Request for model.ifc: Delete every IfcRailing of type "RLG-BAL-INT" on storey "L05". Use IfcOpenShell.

First a look at what the model holds.

```python
import ifcopenshell
import ifcopenshell.util.element

model = ifcopenshell.open("model.ifc")
print(model.schema)
storey = next(s for s in model.by_type("IfcBuildingStorey") if s.Name == "L05")
railings = [e for e in ifcopenshell.util.element.get_decomposition(storey) if e.is_a("IfcRailing")]
seen = {}
for e in railings:
    element_type = ifcopenshell.util.element.get_type(e)
    name = element_type.Name if element_type not in (None, e) else None
    seen[name] = seen.get(name, 0) + 1
for name, count in sorted(seen.items(), key=str):
    print(count, "x", name)
```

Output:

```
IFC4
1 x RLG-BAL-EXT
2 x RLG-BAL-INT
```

```python
import ifcopenshell
import ifcopenshell.api.root
import ifcopenshell.util.element

model = ifcopenshell.open("model.ifc")

storey = next(s for s in model.by_type("IfcBuildingStorey") if s.Name == "L05")
railings = [e for e in ifcopenshell.util.element.get_decomposition(storey) if e.is_a("IfcRailing")]
targets = [e for e in railings if (t := ifcopenshell.util.element.get_type(e)) not in (None, e) and t.Name == "RLG-BAL-INT"]

for e in targets:
    ifcopenshell.api.root.remove_product(model, product=e)
print(len(targets), "removed")

model.write("model_v2.ifc")
```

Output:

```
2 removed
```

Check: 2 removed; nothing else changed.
